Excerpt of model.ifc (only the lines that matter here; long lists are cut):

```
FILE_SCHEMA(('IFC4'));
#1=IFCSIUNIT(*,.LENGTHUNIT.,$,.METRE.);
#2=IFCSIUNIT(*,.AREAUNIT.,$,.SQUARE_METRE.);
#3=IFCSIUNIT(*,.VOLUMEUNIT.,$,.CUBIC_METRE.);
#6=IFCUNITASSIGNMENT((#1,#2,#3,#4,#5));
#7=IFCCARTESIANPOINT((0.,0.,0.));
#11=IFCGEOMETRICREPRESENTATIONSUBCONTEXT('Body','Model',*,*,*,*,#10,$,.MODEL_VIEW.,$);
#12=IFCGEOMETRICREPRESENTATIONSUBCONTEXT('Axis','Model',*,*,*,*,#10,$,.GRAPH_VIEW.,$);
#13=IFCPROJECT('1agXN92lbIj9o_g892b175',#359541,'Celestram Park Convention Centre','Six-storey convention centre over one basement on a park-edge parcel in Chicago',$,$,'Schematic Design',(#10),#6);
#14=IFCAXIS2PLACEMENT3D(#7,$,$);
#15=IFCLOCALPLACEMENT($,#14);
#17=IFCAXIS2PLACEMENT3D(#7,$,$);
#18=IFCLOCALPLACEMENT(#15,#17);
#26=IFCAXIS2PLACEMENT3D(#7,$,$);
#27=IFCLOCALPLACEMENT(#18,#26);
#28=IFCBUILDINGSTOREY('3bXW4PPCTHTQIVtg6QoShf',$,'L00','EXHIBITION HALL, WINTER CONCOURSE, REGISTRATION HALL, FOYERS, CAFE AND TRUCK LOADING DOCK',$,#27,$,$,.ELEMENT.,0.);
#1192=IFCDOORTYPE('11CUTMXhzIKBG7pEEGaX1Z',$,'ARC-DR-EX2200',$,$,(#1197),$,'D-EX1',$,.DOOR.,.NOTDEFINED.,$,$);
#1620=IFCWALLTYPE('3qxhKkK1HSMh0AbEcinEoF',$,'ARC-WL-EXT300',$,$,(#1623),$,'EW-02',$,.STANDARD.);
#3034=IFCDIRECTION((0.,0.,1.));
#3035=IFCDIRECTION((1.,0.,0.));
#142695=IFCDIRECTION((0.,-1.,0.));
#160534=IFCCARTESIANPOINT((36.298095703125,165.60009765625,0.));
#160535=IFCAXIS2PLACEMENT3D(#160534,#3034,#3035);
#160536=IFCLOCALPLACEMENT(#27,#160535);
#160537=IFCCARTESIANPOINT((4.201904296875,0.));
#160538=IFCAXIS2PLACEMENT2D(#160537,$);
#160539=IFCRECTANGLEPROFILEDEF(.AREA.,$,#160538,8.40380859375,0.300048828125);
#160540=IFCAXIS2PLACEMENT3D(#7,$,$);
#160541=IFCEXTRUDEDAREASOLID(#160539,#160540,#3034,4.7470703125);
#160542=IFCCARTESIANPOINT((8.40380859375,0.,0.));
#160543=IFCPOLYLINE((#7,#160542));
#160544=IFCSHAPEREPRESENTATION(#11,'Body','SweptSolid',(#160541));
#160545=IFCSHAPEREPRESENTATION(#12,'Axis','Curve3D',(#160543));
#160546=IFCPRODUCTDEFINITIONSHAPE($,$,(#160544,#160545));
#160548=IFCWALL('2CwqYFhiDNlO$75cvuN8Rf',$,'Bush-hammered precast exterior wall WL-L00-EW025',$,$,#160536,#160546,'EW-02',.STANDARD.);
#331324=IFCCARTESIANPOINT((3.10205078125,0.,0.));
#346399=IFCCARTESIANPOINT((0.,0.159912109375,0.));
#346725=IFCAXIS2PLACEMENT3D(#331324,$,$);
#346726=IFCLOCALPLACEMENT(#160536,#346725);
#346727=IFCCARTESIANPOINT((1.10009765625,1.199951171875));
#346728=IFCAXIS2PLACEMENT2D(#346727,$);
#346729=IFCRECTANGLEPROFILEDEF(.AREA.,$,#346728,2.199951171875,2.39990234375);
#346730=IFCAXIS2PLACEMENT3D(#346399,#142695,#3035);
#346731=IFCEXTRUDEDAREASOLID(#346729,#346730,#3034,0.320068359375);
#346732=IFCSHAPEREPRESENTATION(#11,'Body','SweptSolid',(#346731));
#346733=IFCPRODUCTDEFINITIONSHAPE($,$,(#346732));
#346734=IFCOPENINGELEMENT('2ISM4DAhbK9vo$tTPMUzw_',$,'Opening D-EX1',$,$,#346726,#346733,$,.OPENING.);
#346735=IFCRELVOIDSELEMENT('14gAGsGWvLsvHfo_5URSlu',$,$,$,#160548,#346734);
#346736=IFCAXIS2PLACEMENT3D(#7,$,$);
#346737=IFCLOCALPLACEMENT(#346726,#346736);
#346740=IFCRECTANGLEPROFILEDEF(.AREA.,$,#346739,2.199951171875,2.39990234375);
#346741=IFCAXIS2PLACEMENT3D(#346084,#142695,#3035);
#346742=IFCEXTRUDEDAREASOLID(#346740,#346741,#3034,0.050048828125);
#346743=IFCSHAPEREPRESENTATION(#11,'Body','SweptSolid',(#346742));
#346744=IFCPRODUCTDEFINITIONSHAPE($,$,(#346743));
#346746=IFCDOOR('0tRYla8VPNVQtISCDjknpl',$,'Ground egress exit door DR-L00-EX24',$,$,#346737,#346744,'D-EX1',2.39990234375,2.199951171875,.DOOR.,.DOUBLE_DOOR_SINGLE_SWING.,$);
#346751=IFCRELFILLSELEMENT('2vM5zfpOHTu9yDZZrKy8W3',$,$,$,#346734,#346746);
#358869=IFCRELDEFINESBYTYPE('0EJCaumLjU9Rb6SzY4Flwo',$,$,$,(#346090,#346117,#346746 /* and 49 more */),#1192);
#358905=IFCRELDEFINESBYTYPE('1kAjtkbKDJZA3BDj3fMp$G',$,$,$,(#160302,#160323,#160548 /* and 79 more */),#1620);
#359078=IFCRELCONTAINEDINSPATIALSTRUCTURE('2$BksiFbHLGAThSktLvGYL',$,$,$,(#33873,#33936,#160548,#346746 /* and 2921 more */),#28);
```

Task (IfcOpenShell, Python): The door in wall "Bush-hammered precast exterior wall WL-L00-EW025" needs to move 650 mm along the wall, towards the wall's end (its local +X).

```python
import ifcopenshell
import ifcopenshell.api.geometry
import ifcopenshell.util.placement

model = ifcopenshell.open("model.ifc")

door = model.by_guid("0tRYla8VPNVQtISCDjknpl")
opening = door.FillsVoids[0].RelatingOpeningElement
wall = opening.VoidsElements[0].RelatingBuildingElement

wall_matrix = ifcopenshell.util.placement.get_local_placement(wall.ObjectPlacement)
shift = wall_matrix[:3, 0] * 0.65
before = ifcopenshell.util.placement.get_local_placement(door.ObjectPlacement)[:3, 3].copy()

# The door is placed relative to its opening, so it follows when the opening moves.
matrix = ifcopenshell.util.placement.get_local_placement(opening.ObjectPlacement)
matrix[:3, 3] += shift
ifcopenshell.api.geometry.edit_object_placement(
    model, product=opening, matrix=matrix, is_si=False, should_transform_children=True
)

after = ifcopenshell.util.placement.get_local_placement(door.ObjectPlacement)[:3, 3]
print("door moved by", (after - before).round(3) + 0.0)

model.write("model_v2.ifc")
```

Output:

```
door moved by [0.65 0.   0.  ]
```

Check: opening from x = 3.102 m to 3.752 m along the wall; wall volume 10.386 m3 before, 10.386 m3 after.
